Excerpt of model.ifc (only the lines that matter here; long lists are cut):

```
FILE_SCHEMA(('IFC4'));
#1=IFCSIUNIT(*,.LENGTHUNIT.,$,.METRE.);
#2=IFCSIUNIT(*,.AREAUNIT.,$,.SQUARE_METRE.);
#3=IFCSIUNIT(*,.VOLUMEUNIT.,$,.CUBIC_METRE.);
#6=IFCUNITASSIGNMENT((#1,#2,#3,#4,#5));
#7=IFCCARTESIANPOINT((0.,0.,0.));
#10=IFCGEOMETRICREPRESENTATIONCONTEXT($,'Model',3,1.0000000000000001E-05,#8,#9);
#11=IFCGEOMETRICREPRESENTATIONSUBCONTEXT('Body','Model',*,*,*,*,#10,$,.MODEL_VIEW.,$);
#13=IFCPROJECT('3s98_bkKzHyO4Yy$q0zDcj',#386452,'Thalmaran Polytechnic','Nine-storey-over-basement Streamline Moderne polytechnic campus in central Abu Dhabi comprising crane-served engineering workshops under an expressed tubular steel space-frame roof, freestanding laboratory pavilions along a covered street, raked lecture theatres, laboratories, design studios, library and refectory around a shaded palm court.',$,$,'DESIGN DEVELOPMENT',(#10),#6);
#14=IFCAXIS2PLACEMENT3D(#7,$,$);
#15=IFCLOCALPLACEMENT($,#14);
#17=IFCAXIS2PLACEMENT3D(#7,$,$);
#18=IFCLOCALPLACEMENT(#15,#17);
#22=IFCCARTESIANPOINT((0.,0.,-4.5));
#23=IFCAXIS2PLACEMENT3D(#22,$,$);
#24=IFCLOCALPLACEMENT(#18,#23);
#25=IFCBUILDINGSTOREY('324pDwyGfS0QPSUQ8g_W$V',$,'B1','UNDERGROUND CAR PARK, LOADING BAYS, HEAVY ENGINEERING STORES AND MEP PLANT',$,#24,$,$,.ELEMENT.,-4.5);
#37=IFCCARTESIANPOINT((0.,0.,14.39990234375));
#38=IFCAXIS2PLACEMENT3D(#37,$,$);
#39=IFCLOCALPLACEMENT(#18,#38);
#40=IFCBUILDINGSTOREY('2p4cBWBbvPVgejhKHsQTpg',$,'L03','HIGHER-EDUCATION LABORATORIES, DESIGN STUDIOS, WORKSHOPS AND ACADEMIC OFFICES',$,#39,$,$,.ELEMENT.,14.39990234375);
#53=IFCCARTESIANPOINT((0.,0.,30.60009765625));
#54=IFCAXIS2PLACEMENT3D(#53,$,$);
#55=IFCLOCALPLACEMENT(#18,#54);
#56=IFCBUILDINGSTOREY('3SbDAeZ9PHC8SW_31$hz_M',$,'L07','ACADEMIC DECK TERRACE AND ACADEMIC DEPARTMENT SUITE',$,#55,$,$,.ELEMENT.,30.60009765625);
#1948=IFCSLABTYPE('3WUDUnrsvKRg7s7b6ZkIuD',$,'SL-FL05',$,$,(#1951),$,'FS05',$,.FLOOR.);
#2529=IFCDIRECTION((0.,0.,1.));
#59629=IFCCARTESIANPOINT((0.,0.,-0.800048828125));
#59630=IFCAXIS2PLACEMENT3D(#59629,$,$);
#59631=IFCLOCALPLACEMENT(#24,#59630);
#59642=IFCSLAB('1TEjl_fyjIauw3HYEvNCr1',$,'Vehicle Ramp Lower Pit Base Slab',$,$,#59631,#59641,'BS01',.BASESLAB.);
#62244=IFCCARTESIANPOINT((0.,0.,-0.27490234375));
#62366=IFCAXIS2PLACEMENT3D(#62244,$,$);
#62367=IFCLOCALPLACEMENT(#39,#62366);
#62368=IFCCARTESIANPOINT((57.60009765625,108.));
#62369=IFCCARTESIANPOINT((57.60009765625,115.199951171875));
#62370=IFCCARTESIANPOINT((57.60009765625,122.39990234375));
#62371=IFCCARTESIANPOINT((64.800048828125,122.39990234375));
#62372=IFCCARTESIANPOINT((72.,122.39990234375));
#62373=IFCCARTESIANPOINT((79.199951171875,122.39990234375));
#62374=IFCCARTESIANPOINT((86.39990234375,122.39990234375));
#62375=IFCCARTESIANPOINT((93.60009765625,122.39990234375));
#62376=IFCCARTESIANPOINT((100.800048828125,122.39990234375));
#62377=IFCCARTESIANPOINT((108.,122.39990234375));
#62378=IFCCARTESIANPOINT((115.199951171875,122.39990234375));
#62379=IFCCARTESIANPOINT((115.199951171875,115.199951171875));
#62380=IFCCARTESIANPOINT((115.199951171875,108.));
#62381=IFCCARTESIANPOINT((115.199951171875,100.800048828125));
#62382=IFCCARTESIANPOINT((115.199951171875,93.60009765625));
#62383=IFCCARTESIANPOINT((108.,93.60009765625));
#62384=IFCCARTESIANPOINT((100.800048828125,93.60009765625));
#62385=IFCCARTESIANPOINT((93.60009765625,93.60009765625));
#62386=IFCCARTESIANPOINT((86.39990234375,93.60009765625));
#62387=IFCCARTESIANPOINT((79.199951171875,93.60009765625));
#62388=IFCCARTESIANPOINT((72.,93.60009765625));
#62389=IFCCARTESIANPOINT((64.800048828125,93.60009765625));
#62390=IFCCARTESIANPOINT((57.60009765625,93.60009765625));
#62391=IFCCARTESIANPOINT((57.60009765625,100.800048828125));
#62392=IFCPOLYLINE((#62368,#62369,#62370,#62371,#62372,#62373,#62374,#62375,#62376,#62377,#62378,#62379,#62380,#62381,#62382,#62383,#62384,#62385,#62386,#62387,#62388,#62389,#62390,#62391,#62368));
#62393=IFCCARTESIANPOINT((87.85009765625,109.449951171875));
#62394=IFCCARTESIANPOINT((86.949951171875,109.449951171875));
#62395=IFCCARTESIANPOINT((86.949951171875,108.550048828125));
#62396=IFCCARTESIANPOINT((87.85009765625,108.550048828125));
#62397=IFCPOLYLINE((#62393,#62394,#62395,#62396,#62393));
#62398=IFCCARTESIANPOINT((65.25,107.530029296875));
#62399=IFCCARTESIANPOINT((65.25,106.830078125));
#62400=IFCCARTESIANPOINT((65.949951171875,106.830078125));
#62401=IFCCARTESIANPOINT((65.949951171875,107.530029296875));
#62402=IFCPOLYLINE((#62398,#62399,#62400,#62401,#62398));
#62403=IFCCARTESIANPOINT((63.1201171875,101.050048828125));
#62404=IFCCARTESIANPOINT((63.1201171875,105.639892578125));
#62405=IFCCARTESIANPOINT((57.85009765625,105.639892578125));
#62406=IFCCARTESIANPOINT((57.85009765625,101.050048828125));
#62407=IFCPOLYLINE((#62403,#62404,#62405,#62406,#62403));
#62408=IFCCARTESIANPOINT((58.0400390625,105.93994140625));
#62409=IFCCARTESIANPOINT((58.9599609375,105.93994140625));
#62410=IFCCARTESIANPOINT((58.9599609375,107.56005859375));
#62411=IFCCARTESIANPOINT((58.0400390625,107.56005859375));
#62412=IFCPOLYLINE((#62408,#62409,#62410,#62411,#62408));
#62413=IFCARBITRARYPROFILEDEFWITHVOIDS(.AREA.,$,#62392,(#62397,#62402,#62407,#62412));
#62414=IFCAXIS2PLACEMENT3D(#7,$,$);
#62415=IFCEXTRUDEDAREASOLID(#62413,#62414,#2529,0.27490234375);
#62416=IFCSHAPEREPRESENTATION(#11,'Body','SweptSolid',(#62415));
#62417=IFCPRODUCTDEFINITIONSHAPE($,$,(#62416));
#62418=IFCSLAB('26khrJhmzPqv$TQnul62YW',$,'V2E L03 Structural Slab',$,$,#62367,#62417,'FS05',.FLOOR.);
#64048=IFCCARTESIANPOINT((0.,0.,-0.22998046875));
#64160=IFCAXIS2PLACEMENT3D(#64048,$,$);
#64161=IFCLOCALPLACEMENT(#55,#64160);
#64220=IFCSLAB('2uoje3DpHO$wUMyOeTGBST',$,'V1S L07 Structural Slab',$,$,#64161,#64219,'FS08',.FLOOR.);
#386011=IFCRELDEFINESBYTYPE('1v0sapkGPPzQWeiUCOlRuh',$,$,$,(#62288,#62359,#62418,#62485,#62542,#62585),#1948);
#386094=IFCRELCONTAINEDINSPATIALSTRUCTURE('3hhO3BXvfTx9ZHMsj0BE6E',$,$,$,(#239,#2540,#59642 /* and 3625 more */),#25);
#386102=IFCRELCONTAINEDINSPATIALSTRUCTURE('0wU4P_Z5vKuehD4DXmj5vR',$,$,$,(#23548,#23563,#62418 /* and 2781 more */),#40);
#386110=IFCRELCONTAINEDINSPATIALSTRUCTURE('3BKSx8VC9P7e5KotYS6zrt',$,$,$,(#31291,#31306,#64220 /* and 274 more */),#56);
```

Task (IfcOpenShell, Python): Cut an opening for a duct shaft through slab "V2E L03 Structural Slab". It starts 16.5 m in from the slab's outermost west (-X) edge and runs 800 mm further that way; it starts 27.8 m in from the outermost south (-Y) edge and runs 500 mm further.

```python
import numpy as np
import ifcopenshell
import ifcopenshell.api.feature
import ifcopenshell.api.geometry
import ifcopenshell.api.root
import ifcopenshell.geom
import ifcopenshell.util.placement
import ifcopenshell.util.representation
import ifcopenshell.util.shape
import ifcopenshell.util.unit

model = ifcopenshell.open("model.ifc")
unit_scale = ifcopenshell.util.unit.calculate_unit_scale(model)
settings = ifcopenshell.geom.settings()


def volume(element):
    """Net volume in cubic metres, openings subtracted."""
    shape = ifcopenshell.geom.create_shape(settings, element)
    return ifcopenshell.util.shape.get_volume(shape.geometry)


slab = model.by_guid("26khrJhmzPqv$TQnul62YW")
before = volume(slab)

# Extent in the slab's own axes, in metres. The edges named are its -X and -Y sides.
slab_shape = ifcopenshell.geom.create_shape(settings, slab)
vertices = ifcopenshell.util.shape.get_vertices(slab_shape.geometry)
x_min, y_min, bottom = vertices.min(axis=0)
top = vertices[:, 2].max()

opening = ifcopenshell.api.root.create_entity(model, ifc_class="IfcOpeningElement", name="Duct shaft opening", predefined_type="OPENING")
context = ifcopenshell.util.representation.get_context(model, "Model", "Body", "MODEL_VIEW")
width, depth = 0.8, 0.5
outline = [(0.0, 0.0), (width, 0.0), (width, depth), (0.0, depth), (0.0, 0.0)]
# Overshoot both faces by 50 mm so the cut is clean.
shape = ifcopenshell.api.geometry.add_slab_representation(
    model, context=context, depth=top - bottom + 0.1, polyline=outline
)
ifcopenshell.api.geometry.assign_representation(model, product=opening, representation=shape)

matrix = ifcopenshell.util.placement.get_local_placement(slab.ObjectPlacement)
matrix[:, 3] = matrix @ np.append(np.array([x_min + 16.5, y_min + 27.8, bottom - 0.05]) / unit_scale, 1.0)
ifcopenshell.api.geometry.edit_object_placement(model, product=opening, matrix=matrix, is_si=False)
ifcopenshell.api.feature.add_feature(model, feature=opening, element=slab)

after = volume(slab)

print(f"slab volume {before:.3f} -> {after:.3f} m3")

model.write("model_v2.ifc")
```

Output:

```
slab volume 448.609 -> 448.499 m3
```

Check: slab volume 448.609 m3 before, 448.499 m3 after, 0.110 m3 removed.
